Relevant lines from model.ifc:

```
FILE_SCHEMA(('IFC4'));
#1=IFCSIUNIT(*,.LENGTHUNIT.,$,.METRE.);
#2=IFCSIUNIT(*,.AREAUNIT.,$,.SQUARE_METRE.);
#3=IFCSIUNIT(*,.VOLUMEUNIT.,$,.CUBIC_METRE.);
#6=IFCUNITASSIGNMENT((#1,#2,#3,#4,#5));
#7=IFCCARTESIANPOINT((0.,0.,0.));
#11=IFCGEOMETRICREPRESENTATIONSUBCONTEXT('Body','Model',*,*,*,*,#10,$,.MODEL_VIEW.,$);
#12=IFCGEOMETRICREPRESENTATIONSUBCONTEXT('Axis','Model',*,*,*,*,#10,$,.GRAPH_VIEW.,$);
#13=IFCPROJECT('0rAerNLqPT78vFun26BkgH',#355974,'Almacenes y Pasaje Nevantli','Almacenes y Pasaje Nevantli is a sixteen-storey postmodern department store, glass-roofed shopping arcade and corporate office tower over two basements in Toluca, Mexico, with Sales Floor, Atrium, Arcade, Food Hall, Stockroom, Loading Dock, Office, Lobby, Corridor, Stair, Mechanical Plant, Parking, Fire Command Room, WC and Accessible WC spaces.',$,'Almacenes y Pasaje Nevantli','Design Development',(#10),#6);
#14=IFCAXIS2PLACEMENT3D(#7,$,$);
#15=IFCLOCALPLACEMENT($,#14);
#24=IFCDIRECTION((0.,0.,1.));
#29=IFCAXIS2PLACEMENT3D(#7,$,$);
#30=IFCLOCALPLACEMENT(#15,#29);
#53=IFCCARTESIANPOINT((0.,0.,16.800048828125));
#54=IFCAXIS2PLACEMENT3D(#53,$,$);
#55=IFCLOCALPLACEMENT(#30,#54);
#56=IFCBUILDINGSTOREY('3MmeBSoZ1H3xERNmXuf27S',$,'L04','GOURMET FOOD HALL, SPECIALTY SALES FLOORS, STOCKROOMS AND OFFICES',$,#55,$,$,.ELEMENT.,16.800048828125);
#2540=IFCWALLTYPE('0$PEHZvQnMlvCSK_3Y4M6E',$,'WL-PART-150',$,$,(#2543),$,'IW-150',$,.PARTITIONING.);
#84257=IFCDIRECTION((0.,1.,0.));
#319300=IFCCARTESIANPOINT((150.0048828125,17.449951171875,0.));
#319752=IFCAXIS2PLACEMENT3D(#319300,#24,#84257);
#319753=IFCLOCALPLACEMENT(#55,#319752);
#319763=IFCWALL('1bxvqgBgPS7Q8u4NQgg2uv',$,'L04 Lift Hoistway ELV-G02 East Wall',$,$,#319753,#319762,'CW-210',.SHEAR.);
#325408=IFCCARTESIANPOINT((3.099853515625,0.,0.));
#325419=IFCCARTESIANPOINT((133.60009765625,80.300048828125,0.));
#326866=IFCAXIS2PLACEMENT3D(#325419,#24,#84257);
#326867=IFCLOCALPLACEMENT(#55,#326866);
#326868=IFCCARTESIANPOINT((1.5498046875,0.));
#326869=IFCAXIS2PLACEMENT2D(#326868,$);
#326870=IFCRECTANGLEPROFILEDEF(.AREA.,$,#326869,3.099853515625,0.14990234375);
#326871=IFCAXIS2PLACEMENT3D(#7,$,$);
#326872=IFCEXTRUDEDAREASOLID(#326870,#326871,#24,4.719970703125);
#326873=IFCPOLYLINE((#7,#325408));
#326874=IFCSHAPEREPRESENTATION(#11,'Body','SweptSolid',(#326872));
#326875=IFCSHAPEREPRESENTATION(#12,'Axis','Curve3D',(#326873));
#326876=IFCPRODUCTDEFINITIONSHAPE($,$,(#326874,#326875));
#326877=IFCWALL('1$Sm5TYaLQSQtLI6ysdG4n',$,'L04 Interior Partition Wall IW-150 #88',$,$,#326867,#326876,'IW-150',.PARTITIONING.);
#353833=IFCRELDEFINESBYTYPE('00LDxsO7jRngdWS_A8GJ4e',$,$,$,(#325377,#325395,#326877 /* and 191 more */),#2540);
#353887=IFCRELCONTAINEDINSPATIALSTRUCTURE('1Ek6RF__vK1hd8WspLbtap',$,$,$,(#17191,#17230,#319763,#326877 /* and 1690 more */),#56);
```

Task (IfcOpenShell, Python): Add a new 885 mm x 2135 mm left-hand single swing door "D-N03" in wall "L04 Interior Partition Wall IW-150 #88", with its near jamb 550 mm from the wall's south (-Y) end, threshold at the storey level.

```python
import numpy as np
import ifcopenshell
import ifcopenshell.api.feature
import ifcopenshell.api.geometry
import ifcopenshell.api.root
import ifcopenshell.api.spatial
import ifcopenshell.geom
import ifcopenshell.util.element
import ifcopenshell.util.placement
import ifcopenshell.util.representation
import ifcopenshell.util.shape
import ifcopenshell.util.unit

model = ifcopenshell.open("model.ifc")
unit_scale = ifcopenshell.util.unit.calculate_unit_scale(model)
settings = ifcopenshell.geom.settings()


def volume(element):
    """Net volume in cubic metres, openings subtracted."""
    shape = ifcopenshell.geom.create_shape(settings, element)
    return ifcopenshell.util.shape.get_volume(shape.geometry)


wall = model.by_guid("1$Sm5TYaLQSQtLI6ysdG4n")
storey = ifcopenshell.util.element.get_container(wall, ifc_class="IfcBuildingStorey")
context = ifcopenshell.util.representation.get_context(model, "Model", "Body", "MODEL_VIEW")
before = volume(wall)

width, height, from_end, sill = 0.885, 2.135, 0.55, 0.0  # metres

# The wall runs along its own X axis, and the end named is its -X end.
wall_shape = ifcopenshell.geom.create_shape(settings, wall)
x, y, z = ifcopenshell.util.shape.get_vertices(wall_shape.geometry).T
start = x.min() + from_end
face, thickness = float(y.min()), float(y.max() - y.min())
wall_matrix = ifcopenshell.util.placement.get_local_placement(wall.ObjectPlacement)
level = ifcopenshell.util.placement.get_local_placement(storey.ObjectPlacement)[2, 3]


def in_wall(x, y):
    """Placement at x, y metres in the wall's axes, at sill height."""
    matrix = wall_matrix.copy()
    matrix[:, 3] = wall_matrix @ np.array([x / unit_scale, y / unit_scale, 0.0, 1.0])
    matrix[2, 3] = level + sill / unit_scale
    return matrix


# Opening: a box that overshoots both wall faces by 50 mm.
opening = ifcopenshell.api.root.create_entity(model, ifc_class="IfcOpeningElement", predefined_type="OPENING")
box = ifcopenshell.api.geometry.add_wall_representation(
    model, context=context, length=width, height=height, thickness=thickness + 0.1
)
ifcopenshell.api.geometry.assign_representation(model, product=opening, representation=box)
ifcopenshell.api.geometry.edit_object_placement(model, product=opening, matrix=in_wall(start, face - 0.05), is_si=False)
ifcopenshell.api.feature.add_feature(model, feature=opening, element=wall)

door = ifcopenshell.api.root.create_entity(model, ifc_class="IfcDoor", name="D-N03", predefined_type="DOOR")
door.OverallWidth, door.OverallHeight = width / unit_scale, height / unit_scale
door.OperationType = "SINGLE_SWING_LEFT"
body = ifcopenshell.api.geometry.add_door_representation(
    model,
    context=context,
    overall_width=door.OverallWidth,
    overall_height=door.OverallHeight,
    operation_type="SINGLE_SWING_LEFT",
    lining_properties={"LiningDepth": thickness / unit_scale, "ThresholdDepth": thickness / unit_scale},
)
ifcopenshell.api.geometry.assign_representation(model, product=door, representation=body)
ifcopenshell.api.spatial.assign_container(model, products=[door], relating_structure=storey)
ifcopenshell.api.feature.add_filling(model, opening=opening, element=door)

# The lining spans the wall, so the door starts at the wall face.
ifcopenshell.api.geometry.edit_object_placement(model, product=door, matrix=in_wall(start, face), is_si=False)

after = volume(wall)

print(f"wall volume {before:.3f} -> {after:.3f} m3")

model.write("model_updated.ifc")
```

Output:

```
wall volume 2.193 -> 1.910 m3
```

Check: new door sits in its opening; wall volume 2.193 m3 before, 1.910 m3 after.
